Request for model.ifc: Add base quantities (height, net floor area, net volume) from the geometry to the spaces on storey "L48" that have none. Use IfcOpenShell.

First a look at what the model holds.

```python
import ifcopenshell
import ifcopenshell.util.element
import ifcopenshell.util.unit

model = ifcopenshell.open("model.ifc")
print(model.schema)
for unit_type in ("LENGTHUNIT", "AREAUNIT", "VOLUMEUNIT"):
    print(unit_type, ifcopenshell.util.unit.calculate_unit_scale(model, unit_type))
storey = next(s for s in model.by_type("IfcBuildingStorey") if s.Name == "L48")
spaces = [e for e in ifcopenshell.util.element.get_decomposition(storey) if e.is_a("IfcSpace")]
for e in sorted(spaces, key=lambda e: e.id()):
    print(e.id(), e.is_a(), e.Name, list(ifcopenshell.util.element.get_psets(e, qtos_only=True)), sep=" | ")
```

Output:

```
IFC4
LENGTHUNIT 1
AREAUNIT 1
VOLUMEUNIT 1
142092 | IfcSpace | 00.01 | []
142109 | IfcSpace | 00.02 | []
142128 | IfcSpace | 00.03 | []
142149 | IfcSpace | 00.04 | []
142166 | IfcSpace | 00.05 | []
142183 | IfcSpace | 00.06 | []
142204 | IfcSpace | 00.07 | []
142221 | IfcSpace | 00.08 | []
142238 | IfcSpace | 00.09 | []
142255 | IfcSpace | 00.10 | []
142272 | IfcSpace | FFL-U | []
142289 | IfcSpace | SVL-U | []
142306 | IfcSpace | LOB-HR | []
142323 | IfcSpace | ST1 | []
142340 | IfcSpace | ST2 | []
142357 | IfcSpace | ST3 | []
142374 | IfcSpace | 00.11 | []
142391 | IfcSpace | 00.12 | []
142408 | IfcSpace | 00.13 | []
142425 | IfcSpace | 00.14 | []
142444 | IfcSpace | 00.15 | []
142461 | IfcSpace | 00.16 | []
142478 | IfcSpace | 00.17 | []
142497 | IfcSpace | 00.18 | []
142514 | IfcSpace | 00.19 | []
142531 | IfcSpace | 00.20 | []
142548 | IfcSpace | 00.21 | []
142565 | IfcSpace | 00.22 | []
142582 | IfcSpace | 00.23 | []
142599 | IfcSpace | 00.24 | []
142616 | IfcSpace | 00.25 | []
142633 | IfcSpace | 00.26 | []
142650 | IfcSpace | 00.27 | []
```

```python
import ifcopenshell
import ifcopenshell.api.pset
import ifcopenshell.geom
import ifcopenshell.util.element
import ifcopenshell.util.shape
import ifcopenshell.util.unit

model = ifcopenshell.open("model.ifc")
unit_scale = ifcopenshell.util.unit.calculate_unit_scale(model)
area_scale = ifcopenshell.util.unit.calculate_unit_scale(model, "AREAUNIT")
volume_scale = ifcopenshell.util.unit.calculate_unit_scale(model, "VOLUMEUNIT")
settings = ifcopenshell.geom.settings()

storey = next(s for s in model.by_type("IfcBuildingStorey") if s.Name == "L48")
spaces = [e for e in ifcopenshell.util.element.get_decomposition(storey) if e.is_a("IfcSpace")]

for e in sorted(spaces, key=lambda e: e.id()):
    if ifcopenshell.util.element.get_psets(e, qtos_only=True, should_inherit=False):
        continue
    # Geometry comes back in metres, in the element's own axes.
    shape = ifcopenshell.geom.create_shape(settings, e)
    values = {
        "Height": ifcopenshell.util.shape.get_z(shape.geometry) / unit_scale,
        "NetFloorArea": ifcopenshell.util.shape.get_footprint_area(shape.geometry) / area_scale,
        "NetVolume": ifcopenshell.util.shape.get_volume(shape.geometry) / volume_scale,
    }
    qto = ifcopenshell.api.pset.add_qto(model, product=e, name="Qto_SpaceBaseQuantities")
    ifcopenshell.api.pset.edit_qto(model, qto=qto, properties=values)
    print(e.id(), {k: round(v, 3) for k, v in values.items()})

model.write("model_rev.ifc")
```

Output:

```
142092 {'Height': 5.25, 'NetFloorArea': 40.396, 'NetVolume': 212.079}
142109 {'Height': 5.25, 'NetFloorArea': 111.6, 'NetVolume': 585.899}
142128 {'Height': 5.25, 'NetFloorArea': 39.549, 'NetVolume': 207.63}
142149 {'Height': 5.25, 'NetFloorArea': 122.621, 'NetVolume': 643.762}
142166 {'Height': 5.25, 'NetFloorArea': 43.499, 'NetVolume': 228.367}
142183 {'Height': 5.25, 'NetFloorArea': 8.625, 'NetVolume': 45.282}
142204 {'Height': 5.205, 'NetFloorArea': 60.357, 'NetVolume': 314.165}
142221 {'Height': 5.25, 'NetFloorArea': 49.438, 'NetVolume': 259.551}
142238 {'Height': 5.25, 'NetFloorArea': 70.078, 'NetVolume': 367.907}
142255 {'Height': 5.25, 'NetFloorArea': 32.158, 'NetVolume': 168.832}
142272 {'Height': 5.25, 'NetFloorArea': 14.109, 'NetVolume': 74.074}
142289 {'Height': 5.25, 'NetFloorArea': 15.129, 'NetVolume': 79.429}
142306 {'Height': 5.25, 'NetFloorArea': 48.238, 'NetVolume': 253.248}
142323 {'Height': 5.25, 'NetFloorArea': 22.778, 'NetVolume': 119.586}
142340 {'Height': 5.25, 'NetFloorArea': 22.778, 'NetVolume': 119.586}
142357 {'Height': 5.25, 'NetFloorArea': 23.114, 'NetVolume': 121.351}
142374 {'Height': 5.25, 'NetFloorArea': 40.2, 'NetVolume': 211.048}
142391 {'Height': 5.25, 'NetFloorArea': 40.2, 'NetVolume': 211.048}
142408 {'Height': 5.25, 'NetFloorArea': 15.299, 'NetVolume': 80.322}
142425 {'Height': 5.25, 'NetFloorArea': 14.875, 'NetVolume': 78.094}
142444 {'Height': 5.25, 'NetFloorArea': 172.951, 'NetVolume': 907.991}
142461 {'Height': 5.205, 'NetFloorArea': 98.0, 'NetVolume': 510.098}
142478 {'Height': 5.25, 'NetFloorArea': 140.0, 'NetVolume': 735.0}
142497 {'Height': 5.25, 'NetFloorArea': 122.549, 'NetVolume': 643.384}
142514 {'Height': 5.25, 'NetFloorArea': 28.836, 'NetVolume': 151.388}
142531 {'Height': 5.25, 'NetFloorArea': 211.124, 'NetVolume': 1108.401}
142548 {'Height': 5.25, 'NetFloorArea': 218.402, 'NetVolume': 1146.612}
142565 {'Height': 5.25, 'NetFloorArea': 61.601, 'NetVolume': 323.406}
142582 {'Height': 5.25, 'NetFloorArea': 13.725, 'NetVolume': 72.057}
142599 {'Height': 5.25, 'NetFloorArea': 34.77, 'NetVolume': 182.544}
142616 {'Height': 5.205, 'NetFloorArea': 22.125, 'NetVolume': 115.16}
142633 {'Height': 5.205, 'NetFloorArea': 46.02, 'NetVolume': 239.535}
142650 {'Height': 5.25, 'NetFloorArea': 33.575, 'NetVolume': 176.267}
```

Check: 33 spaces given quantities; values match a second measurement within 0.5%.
